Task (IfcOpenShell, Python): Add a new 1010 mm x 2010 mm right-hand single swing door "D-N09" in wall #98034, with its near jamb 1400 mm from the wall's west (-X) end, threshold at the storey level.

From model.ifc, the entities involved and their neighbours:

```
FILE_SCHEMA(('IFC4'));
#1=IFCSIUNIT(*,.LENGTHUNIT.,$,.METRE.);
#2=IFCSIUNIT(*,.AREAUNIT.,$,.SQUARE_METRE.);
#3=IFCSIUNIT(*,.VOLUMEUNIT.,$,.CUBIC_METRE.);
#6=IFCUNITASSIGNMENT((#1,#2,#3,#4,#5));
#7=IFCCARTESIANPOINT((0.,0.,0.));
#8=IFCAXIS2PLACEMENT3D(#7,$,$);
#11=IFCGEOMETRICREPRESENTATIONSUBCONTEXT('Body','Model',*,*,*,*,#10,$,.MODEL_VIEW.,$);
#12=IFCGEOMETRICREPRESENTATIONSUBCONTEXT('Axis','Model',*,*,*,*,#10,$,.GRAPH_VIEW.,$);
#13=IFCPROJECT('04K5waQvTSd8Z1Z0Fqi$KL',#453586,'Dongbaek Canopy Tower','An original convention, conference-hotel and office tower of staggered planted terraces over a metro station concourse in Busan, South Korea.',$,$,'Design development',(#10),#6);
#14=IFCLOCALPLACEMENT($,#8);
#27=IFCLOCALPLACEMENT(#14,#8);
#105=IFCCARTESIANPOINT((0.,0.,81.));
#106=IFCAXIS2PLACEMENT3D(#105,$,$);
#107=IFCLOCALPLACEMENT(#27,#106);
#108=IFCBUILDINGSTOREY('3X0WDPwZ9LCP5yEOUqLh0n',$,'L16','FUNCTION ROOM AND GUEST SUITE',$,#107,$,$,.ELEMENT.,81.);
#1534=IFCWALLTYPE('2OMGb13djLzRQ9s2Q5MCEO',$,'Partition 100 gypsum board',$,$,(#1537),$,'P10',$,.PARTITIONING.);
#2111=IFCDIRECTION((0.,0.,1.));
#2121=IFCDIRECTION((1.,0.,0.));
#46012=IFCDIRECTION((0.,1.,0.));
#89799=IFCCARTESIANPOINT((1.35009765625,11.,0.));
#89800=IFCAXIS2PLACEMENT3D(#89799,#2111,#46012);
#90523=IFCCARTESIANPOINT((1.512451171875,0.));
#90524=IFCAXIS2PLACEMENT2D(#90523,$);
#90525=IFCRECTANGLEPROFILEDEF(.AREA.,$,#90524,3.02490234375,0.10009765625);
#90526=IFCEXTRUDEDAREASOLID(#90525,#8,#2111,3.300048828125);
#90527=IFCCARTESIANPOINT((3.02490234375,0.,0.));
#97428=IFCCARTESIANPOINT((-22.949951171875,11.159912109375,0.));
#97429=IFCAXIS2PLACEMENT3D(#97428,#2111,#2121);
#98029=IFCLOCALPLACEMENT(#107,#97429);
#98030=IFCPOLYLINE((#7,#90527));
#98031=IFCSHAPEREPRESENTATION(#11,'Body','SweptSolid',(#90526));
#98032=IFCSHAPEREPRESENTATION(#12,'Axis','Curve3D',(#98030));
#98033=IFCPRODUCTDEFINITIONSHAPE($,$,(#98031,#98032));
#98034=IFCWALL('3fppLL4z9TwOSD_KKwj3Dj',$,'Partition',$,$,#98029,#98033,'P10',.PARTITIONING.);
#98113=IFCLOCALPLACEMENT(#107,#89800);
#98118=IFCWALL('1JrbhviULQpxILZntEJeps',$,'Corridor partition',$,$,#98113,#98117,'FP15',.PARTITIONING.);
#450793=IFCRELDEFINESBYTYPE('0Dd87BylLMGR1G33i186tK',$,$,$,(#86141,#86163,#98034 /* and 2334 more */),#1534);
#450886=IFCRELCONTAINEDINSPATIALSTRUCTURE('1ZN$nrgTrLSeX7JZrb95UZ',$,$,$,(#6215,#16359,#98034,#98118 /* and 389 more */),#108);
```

```python
import numpy as np
import ifcopenshell
import ifcopenshell.api.feature
import ifcopenshell.api.geometry
import ifcopenshell.api.root
import ifcopenshell.api.spatial
import ifcopenshell.geom
import ifcopenshell.util.element
import ifcopenshell.util.placement
import ifcopenshell.util.representation
import ifcopenshell.util.shape
import ifcopenshell.util.unit

model = ifcopenshell.open("model.ifc")
unit_scale = ifcopenshell.util.unit.calculate_unit_scale(model)
settings = ifcopenshell.geom.settings()


def volume(element):
    """Net volume in cubic metres, openings subtracted."""
    shape = ifcopenshell.geom.create_shape(settings, element)
    return ifcopenshell.util.shape.get_volume(shape.geometry)


wall = model.by_guid("3fppLL4z9TwOSD_KKwj3Dj")
storey = ifcopenshell.util.element.get_container(wall, ifc_class="IfcBuildingStorey")
context = ifcopenshell.util.representation.get_context(model, "Model", "Body", "MODEL_VIEW")
before = volume(wall)

width, height, from_end, sill = 1.01, 2.01, 1.4, 0.0  # metres

# The wall runs along its own X axis, and the end named is its -X end.
wall_shape = ifcopenshell.geom.create_shape(settings, wall)
x, y, z = ifcopenshell.util.shape.get_vertices(wall_shape.geometry).T
start = x.min() + from_end
face, thickness = float(y.min()), float(y.max() - y.min())
wall_matrix = ifcopenshell.util.placement.get_local_placement(wall.ObjectPlacement)
level = ifcopenshell.util.placement.get_local_placement(storey.ObjectPlacement)[2, 3]


def in_wall(x, y):
    """Placement at x, y metres in the wall's axes, at sill height."""
    matrix = wall_matrix.copy()
    matrix[:, 3] = wall_matrix @ np.array([x / unit_scale, y / unit_scale, 0.0, 1.0])
    matrix[2, 3] = level + sill / unit_scale
    return matrix


# Opening: a box that overshoots both wall faces by 50 mm.
opening = ifcopenshell.api.root.create_entity(model, ifc_class="IfcOpeningElement", predefined_type="OPENING")
box = ifcopenshell.api.geometry.add_wall_representation(
    model, context=context, length=width, height=height, thickness=thickness + 0.1
)
ifcopenshell.api.geometry.assign_representation(model, product=opening, representation=box)
ifcopenshell.api.geometry.edit_object_placement(model, product=opening, matrix=in_wall(start, face - 0.05), is_si=False)
ifcopenshell.api.feature.add_feature(model, feature=opening, element=wall)

door = ifcopenshell.api.root.create_entity(model, ifc_class="IfcDoor", name="D-N09", predefined_type="DOOR")
door.OverallWidth, door.OverallHeight = width / unit_scale, height / unit_scale
door.OperationType = "SINGLE_SWING_RIGHT"
body = ifcopenshell.api.geometry.add_door_representation(
    model,
    context=context,
    overall_width=door.OverallWidth,
    overall_height=door.OverallHeight,
    operation_type="SINGLE_SWING_RIGHT",
    lining_properties={"LiningDepth": thickness / unit_scale, "ThresholdDepth": thickness / unit_scale},
)
ifcopenshell.api.geometry.assign_representation(model, product=door, representation=body)
ifcopenshell.api.spatial.assign_container(model, products=[door], relating_structure=storey)
ifcopenshell.api.feature.add_filling(model, opening=opening, element=door)

# The lining spans the wall, so the door starts at the wall face.
ifcopenshell.api.geometry.edit_object_placement(model, product=door, matrix=in_wall(start, face), is_si=False)

after = volume(wall)

print(f"wall volume {before:.3f} -> {after:.3f} m3")

model.write("model_v2.ifc")
```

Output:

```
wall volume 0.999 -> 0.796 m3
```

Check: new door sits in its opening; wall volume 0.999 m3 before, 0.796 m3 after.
